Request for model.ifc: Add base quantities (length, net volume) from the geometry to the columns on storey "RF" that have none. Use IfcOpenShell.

First a look at what the model holds.

```python
import ifcopenshell
import ifcopenshell.util.element
import ifcopenshell.util.unit

model = ifcopenshell.open("model.ifc")
print(model.schema)
for unit_type in ("LENGTHUNIT", "AREAUNIT", "VOLUMEUNIT"):
    print(unit_type, ifcopenshell.util.unit.calculate_unit_scale(model, unit_type))
storey = next(s for s in model.by_type("IfcBuildingStorey") if s.Name == "RF")
columns = [e for e in ifcopenshell.util.element.get_decomposition(storey) if e.is_a("IfcColumn")]
for e in sorted(columns, key=lambda e: e.id()):
    print(e.id(), e.is_a(), e.Name, list(ifcopenshell.util.element.get_psets(e, qtos_only=True)), sep=" | ")
```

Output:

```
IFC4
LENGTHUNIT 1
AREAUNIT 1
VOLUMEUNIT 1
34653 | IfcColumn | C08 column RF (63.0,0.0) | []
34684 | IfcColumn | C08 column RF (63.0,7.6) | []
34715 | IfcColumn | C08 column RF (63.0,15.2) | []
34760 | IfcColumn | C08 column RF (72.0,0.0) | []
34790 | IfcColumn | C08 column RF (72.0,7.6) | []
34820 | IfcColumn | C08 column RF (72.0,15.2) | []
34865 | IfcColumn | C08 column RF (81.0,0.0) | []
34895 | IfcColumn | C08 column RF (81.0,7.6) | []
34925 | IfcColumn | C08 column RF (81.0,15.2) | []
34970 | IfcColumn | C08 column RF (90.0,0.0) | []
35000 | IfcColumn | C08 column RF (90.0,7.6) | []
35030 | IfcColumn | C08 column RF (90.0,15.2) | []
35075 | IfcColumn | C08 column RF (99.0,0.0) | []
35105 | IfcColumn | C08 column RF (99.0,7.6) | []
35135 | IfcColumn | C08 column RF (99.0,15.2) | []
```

```python
import ifcopenshell
import ifcopenshell.api.pset
import ifcopenshell.geom
import ifcopenshell.util.element
import ifcopenshell.util.shape
import ifcopenshell.util.unit

model = ifcopenshell.open("model.ifc")
unit_scale = ifcopenshell.util.unit.calculate_unit_scale(model)
volume_scale = ifcopenshell.util.unit.calculate_unit_scale(model, "VOLUMEUNIT")
settings = ifcopenshell.geom.settings()

storey = next(s for s in model.by_type("IfcBuildingStorey") if s.Name == "RF")
columns = [e for e in ifcopenshell.util.element.get_decomposition(storey) if e.is_a("IfcColumn")]

for e in sorted(columns, key=lambda e: e.id()):
    if ifcopenshell.util.element.get_psets(e, qtos_only=True, should_inherit=False):
        continue
    # Geometry comes back in metres, in the element's own axes.
    shape = ifcopenshell.geom.create_shape(settings, e)
    values = {
        "Length": ifcopenshell.util.shape.get_z(shape.geometry) / unit_scale,
        "NetVolume": ifcopenshell.util.shape.get_volume(shape.geometry) / volume_scale,
    }
    qto = ifcopenshell.api.pset.add_qto(model, product=e, name="Qto_ColumnBaseQuantities")
    ifcopenshell.api.pset.edit_qto(model, qto=qto, properties=values)
    print(e.id(), {k: round(v, 3) for k, v in values.items()})

model.write("model_updated.ifc")
```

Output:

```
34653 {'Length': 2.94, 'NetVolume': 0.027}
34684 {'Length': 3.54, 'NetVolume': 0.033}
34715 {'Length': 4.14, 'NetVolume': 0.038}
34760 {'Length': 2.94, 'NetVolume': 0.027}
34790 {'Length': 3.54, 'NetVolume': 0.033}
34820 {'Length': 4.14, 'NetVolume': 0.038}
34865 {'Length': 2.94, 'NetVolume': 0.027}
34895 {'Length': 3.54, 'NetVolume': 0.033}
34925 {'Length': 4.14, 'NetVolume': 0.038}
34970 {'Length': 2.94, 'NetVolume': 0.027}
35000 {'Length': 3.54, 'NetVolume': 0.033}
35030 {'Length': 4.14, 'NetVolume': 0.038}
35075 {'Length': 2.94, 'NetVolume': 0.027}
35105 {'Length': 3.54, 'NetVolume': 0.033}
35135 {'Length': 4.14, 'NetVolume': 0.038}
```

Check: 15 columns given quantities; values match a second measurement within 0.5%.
